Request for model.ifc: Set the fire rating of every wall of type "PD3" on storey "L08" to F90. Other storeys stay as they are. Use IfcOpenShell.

First a look at what the model holds.

```python
import ifcopenshell
import ifcopenshell.util.element

model = ifcopenshell.open("model.ifc")
print(model.schema)
storey = next(s for s in model.by_type("IfcBuildingStorey") if s.Name == "L08")
walls = [e for e in ifcopenshell.util.element.get_decomposition(storey) if e.is_a("IfcWall")]
seen = {}
for e in walls:
    element_type = ifcopenshell.util.element.get_type(e)
    key = (element_type.Name if element_type != e and element_type else None, ifcopenshell.util.element.get_pset(e, "Pset_WallCommon", "FireRating"))
    seen[key] = seen.get(key, 0) + 1
for (name, value), count in sorted(seen.items(), key=str):
    print(count, "x", name, "|", value)
```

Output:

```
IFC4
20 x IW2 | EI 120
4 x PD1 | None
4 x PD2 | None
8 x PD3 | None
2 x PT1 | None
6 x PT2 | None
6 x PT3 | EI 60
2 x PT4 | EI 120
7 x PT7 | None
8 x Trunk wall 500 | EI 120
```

```python
import ifcopenshell
import ifcopenshell.api.pset
import ifcopenshell.util.element

model = ifcopenshell.open("model.ifc")

storey = next(s for s in model.by_type("IfcBuildingStorey") if s.Name == "L08")
walls = [e for e in ifcopenshell.util.element.get_decomposition(storey) if e.is_a("IfcWall")]

count = 0
for e in walls:
    element_type = ifcopenshell.util.element.get_type(e)
    if element_type in (None, e) or element_type.Name != "PD3":
        continue
    # add_pset returns the element's existing set when there is one.
    pset = ifcopenshell.api.pset.add_pset(model, product=e, name="Pset_WallCommon")
    ifcopenshell.api.pset.edit_pset(model, pset=pset, properties={"FireRating": "F90"})
    count += 1

print(count, "walls updated")

model.write("model_edited.ifc")
```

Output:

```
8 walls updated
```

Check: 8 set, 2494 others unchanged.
